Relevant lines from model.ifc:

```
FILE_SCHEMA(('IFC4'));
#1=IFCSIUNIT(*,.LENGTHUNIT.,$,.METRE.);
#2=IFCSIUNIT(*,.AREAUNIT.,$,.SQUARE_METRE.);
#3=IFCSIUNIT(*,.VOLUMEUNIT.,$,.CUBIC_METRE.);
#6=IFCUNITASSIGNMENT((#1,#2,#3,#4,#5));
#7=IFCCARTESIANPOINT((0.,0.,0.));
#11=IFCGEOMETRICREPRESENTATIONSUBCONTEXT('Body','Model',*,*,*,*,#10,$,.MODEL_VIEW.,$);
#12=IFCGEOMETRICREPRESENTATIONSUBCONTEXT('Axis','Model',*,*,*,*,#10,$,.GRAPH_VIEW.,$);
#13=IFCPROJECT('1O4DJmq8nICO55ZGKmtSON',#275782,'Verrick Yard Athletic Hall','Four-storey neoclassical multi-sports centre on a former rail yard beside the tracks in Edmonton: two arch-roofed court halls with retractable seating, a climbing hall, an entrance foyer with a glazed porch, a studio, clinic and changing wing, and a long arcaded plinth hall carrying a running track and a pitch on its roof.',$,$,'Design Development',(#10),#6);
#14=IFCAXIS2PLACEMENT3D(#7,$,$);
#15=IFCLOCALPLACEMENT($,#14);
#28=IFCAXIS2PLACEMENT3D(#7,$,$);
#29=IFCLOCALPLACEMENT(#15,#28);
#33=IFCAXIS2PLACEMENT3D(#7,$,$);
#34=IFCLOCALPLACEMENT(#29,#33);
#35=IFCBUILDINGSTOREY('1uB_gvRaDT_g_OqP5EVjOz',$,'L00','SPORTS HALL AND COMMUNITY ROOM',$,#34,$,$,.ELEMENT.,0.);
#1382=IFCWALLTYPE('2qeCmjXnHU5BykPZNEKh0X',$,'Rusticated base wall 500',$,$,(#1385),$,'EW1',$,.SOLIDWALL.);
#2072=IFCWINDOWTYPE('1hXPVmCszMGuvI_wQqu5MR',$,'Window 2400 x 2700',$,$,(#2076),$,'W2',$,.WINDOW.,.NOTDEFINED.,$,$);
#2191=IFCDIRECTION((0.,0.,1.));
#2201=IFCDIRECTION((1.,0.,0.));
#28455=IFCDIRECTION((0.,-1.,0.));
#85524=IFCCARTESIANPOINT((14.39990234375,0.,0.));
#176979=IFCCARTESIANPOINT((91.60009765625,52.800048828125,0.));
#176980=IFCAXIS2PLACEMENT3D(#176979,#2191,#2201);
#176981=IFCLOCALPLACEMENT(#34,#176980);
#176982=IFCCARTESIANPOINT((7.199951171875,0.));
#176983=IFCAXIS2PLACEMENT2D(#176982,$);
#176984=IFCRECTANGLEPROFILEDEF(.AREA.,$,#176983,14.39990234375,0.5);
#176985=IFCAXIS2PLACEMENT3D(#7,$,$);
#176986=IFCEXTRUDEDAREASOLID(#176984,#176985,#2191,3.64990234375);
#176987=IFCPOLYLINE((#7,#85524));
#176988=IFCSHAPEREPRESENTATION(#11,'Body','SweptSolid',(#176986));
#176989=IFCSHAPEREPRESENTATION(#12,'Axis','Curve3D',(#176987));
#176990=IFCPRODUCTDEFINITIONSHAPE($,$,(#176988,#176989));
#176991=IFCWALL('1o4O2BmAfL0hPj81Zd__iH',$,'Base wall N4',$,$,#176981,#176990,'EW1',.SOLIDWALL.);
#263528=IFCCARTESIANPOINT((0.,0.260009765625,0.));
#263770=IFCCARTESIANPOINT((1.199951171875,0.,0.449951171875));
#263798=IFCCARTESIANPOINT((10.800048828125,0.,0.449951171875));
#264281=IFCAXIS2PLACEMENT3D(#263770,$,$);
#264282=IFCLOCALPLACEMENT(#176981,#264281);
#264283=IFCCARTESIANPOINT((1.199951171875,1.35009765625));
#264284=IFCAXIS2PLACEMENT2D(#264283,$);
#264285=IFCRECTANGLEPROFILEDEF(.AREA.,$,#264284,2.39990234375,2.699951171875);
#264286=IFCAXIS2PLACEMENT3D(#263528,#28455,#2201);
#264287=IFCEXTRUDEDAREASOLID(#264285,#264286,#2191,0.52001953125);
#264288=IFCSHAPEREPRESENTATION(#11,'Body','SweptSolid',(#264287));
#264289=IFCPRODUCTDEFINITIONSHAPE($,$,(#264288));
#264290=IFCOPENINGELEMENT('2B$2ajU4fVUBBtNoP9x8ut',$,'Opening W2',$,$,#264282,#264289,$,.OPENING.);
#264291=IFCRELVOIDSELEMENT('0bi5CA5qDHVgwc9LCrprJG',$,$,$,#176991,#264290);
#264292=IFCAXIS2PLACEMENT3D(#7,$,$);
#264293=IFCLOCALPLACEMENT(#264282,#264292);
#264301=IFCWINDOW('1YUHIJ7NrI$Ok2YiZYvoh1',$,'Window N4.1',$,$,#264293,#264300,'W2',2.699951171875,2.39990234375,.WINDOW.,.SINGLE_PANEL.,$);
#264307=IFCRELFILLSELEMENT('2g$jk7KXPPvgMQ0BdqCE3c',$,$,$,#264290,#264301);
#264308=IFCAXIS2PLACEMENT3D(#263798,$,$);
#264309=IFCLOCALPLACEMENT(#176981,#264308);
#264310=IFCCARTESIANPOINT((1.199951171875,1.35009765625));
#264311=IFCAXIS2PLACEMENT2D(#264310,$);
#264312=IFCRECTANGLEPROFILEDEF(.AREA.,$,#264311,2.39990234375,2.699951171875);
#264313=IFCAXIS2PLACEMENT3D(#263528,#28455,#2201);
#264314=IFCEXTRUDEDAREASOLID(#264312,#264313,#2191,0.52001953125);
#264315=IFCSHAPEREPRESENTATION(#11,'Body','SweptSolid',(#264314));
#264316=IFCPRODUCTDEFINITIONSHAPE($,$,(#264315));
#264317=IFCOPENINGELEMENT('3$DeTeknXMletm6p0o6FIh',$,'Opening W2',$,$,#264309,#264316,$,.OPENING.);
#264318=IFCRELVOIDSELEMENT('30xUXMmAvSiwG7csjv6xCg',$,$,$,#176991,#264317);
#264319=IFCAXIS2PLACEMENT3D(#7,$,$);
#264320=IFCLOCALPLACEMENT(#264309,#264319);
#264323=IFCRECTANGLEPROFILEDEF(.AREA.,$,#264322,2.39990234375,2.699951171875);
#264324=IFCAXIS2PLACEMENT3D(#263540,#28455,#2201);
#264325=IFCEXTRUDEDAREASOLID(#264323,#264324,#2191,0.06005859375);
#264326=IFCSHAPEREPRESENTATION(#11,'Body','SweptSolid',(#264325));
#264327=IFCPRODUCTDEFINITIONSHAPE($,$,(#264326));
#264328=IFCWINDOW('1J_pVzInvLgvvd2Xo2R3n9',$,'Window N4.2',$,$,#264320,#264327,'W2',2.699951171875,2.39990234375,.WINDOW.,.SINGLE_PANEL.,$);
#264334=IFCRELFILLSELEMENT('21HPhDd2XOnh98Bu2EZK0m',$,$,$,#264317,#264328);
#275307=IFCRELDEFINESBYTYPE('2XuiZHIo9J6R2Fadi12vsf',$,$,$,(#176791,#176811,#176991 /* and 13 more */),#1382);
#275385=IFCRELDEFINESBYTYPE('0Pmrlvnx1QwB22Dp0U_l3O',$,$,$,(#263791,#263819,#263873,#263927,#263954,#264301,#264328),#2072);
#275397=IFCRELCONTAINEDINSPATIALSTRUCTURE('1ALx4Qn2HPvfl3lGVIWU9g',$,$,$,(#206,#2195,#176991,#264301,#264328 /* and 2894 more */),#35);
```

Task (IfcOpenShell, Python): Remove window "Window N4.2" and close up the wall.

```python
import ifcopenshell
import ifcopenshell.api.feature
import ifcopenshell.api.root
import ifcopenshell.geom
import ifcopenshell.util.shape

model = ifcopenshell.open("model.ifc")
settings = ifcopenshell.geom.settings()


def volume(element):
    """Net volume in cubic metres, openings subtracted."""
    shape = ifcopenshell.geom.create_shape(settings, element)
    return ifcopenshell.util.shape.get_volume(shape.geometry)


window = model.by_guid("1J_pVzInvLgvvd2Xo2R3n9")
opening = window.FillsVoids[0].RelatingOpeningElement
wall = opening.VoidsElements[0].RelatingBuildingElement
before = volume(wall)

ifcopenshell.api.root.remove_product(model, product=window)
ifcopenshell.api.feature.remove_feature(model, feature=opening)

after = volume(wall)

print(f"wall volume {before:.3f} -> {after:.3f} m3")

model.write("model_edited.ifc")
```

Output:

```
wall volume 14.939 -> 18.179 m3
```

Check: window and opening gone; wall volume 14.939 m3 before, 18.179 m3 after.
